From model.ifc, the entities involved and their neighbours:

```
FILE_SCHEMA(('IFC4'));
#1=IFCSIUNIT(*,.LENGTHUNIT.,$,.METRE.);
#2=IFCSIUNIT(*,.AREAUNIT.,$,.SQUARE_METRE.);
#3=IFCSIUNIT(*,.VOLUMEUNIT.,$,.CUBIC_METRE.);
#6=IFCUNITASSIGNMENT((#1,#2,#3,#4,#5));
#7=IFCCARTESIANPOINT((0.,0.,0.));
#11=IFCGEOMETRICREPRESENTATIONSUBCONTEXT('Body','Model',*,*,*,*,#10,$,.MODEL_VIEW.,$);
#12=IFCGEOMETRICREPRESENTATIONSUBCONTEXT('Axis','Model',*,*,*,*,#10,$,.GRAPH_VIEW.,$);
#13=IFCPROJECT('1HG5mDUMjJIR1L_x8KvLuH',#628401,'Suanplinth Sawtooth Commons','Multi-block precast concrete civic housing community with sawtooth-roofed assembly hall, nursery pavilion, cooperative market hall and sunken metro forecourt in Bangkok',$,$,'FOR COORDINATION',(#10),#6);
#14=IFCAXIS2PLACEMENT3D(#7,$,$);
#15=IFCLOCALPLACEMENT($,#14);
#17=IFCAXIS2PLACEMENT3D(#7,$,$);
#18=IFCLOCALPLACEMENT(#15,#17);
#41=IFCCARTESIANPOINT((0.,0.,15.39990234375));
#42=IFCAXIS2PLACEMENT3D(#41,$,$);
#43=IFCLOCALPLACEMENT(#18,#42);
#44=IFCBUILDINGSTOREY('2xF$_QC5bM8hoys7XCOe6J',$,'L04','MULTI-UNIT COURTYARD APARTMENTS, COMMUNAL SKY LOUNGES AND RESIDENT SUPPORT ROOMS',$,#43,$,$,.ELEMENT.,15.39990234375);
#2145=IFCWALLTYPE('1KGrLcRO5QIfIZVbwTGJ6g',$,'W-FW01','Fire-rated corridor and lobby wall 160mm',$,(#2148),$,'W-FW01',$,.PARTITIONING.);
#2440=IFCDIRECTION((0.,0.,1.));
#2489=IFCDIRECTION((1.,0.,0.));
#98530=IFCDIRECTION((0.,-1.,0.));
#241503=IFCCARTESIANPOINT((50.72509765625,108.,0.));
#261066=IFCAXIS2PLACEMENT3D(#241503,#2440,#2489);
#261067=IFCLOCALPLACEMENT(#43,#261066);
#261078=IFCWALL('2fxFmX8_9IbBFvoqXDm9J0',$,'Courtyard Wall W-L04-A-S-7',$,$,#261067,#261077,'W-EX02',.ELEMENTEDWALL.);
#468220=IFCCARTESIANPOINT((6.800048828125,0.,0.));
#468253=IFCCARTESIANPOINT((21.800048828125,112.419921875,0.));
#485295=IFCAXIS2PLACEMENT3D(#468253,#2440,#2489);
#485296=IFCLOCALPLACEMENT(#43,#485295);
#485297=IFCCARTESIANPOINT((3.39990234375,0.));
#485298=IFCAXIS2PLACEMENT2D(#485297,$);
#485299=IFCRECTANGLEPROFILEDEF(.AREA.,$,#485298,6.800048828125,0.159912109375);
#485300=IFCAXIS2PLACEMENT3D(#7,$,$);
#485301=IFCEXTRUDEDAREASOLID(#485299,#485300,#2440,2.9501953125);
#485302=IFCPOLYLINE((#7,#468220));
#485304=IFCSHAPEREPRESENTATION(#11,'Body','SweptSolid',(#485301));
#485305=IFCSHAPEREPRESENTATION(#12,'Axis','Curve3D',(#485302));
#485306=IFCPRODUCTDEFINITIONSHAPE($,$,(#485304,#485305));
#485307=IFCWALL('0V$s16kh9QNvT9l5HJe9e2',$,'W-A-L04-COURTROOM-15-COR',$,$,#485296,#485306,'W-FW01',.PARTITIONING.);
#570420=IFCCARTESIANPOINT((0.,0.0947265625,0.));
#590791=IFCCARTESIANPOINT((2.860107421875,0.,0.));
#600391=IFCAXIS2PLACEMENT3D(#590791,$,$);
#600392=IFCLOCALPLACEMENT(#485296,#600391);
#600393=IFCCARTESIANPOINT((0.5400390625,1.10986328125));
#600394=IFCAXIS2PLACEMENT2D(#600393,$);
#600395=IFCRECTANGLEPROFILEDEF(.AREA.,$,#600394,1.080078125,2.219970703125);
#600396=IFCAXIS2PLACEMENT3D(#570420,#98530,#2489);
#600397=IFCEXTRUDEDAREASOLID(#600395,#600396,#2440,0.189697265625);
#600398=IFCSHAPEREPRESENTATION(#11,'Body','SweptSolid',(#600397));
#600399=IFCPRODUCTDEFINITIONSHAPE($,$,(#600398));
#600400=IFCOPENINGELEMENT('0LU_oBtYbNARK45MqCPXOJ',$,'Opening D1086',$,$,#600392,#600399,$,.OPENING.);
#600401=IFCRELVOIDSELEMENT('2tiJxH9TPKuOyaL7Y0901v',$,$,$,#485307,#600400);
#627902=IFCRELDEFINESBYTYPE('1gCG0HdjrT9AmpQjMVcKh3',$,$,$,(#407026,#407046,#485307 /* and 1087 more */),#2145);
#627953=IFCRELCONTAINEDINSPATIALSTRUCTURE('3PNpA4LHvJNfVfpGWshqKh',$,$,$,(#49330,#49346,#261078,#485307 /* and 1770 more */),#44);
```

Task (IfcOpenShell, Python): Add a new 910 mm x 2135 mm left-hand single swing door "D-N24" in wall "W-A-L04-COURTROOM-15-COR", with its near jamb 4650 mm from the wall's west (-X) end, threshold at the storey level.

```python
import numpy as np
import ifcopenshell
import ifcopenshell.api.feature
import ifcopenshell.api.geometry
import ifcopenshell.api.root
import ifcopenshell.api.spatial
import ifcopenshell.geom
import ifcopenshell.util.element
import ifcopenshell.util.placement
import ifcopenshell.util.representation
import ifcopenshell.util.shape
import ifcopenshell.util.unit

model = ifcopenshell.open("model.ifc")
unit_scale = ifcopenshell.util.unit.calculate_unit_scale(model)
settings = ifcopenshell.geom.settings()


def volume(element):
    """Net volume in cubic metres, openings subtracted."""
    shape = ifcopenshell.geom.create_shape(settings, element)
    return ifcopenshell.util.shape.get_volume(shape.geometry)


wall = model.by_guid("0V$s16kh9QNvT9l5HJe9e2")
storey = ifcopenshell.util.element.get_container(wall, ifc_class="IfcBuildingStorey")
context = ifcopenshell.util.representation.get_context(model, "Model", "Body", "MODEL_VIEW")
before = volume(wall)

width, height, from_end, sill = 0.91, 2.135, 4.65, 0.0  # metres

# The wall runs along its own X axis, and the end named is its -X end.
wall_shape = ifcopenshell.geom.create_shape(settings, wall)
x, y, z = ifcopenshell.util.shape.get_vertices(wall_shape.geometry).T
start = x.min() + from_end
face, thickness = float(y.min()), float(y.max() - y.min())
wall_matrix = ifcopenshell.util.placement.get_local_placement(wall.ObjectPlacement)
level = ifcopenshell.util.placement.get_local_placement(storey.ObjectPlacement)[2, 3]


def in_wall(x, y):
    """Placement at x, y metres in the wall's axes, at sill height."""
    matrix = wall_matrix.copy()
    matrix[:, 3] = wall_matrix @ np.array([x / unit_scale, y / unit_scale, 0.0, 1.0])
    matrix[2, 3] = level + sill / unit_scale
    return matrix


# Opening: a box that overshoots both wall faces by 50 mm.
opening = ifcopenshell.api.root.create_entity(model, ifc_class="IfcOpeningElement", predefined_type="OPENING")
box = ifcopenshell.api.geometry.add_wall_representation(
    model, context=context, length=width, height=height, thickness=thickness + 0.1
)
ifcopenshell.api.geometry.assign_representation(model, product=opening, representation=box)
ifcopenshell.api.geometry.edit_object_placement(model, product=opening, matrix=in_wall(start, face - 0.05), is_si=False)
ifcopenshell.api.feature.add_feature(model, feature=opening, element=wall)

door = ifcopenshell.api.root.create_entity(model, ifc_class="IfcDoor", name="D-N24", predefined_type="DOOR")
door.OverallWidth, door.OverallHeight = width / unit_scale, height / unit_scale
door.OperationType = "SINGLE_SWING_LEFT"
body = ifcopenshell.api.geometry.add_door_representation(
    model,
    context=context,
    overall_width=door.OverallWidth,
    overall_height=door.OverallHeight,
    operation_type="SINGLE_SWING_LEFT",
    lining_properties={"LiningDepth": thickness / unit_scale, "ThresholdDepth": thickness / unit_scale},
)
ifcopenshell.api.geometry.assign_representation(model, product=door, representation=body)
ifcopenshell.api.spatial.assign_container(model, products=[door], relating_structure=storey)
ifcopenshell.api.feature.add_filling(model, opening=opening, element=door)

# The lining spans the wall, so the door starts at the wall face.
ifcopenshell.api.geometry.edit_object_placement(model, product=door, matrix=in_wall(start, face), is_si=False)

after = volume(wall)

print(f"wall volume {before:.3f} -> {after:.3f} m3")

model.write("model_edited.ifc")
```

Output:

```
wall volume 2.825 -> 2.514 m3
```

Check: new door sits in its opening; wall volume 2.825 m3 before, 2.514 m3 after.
